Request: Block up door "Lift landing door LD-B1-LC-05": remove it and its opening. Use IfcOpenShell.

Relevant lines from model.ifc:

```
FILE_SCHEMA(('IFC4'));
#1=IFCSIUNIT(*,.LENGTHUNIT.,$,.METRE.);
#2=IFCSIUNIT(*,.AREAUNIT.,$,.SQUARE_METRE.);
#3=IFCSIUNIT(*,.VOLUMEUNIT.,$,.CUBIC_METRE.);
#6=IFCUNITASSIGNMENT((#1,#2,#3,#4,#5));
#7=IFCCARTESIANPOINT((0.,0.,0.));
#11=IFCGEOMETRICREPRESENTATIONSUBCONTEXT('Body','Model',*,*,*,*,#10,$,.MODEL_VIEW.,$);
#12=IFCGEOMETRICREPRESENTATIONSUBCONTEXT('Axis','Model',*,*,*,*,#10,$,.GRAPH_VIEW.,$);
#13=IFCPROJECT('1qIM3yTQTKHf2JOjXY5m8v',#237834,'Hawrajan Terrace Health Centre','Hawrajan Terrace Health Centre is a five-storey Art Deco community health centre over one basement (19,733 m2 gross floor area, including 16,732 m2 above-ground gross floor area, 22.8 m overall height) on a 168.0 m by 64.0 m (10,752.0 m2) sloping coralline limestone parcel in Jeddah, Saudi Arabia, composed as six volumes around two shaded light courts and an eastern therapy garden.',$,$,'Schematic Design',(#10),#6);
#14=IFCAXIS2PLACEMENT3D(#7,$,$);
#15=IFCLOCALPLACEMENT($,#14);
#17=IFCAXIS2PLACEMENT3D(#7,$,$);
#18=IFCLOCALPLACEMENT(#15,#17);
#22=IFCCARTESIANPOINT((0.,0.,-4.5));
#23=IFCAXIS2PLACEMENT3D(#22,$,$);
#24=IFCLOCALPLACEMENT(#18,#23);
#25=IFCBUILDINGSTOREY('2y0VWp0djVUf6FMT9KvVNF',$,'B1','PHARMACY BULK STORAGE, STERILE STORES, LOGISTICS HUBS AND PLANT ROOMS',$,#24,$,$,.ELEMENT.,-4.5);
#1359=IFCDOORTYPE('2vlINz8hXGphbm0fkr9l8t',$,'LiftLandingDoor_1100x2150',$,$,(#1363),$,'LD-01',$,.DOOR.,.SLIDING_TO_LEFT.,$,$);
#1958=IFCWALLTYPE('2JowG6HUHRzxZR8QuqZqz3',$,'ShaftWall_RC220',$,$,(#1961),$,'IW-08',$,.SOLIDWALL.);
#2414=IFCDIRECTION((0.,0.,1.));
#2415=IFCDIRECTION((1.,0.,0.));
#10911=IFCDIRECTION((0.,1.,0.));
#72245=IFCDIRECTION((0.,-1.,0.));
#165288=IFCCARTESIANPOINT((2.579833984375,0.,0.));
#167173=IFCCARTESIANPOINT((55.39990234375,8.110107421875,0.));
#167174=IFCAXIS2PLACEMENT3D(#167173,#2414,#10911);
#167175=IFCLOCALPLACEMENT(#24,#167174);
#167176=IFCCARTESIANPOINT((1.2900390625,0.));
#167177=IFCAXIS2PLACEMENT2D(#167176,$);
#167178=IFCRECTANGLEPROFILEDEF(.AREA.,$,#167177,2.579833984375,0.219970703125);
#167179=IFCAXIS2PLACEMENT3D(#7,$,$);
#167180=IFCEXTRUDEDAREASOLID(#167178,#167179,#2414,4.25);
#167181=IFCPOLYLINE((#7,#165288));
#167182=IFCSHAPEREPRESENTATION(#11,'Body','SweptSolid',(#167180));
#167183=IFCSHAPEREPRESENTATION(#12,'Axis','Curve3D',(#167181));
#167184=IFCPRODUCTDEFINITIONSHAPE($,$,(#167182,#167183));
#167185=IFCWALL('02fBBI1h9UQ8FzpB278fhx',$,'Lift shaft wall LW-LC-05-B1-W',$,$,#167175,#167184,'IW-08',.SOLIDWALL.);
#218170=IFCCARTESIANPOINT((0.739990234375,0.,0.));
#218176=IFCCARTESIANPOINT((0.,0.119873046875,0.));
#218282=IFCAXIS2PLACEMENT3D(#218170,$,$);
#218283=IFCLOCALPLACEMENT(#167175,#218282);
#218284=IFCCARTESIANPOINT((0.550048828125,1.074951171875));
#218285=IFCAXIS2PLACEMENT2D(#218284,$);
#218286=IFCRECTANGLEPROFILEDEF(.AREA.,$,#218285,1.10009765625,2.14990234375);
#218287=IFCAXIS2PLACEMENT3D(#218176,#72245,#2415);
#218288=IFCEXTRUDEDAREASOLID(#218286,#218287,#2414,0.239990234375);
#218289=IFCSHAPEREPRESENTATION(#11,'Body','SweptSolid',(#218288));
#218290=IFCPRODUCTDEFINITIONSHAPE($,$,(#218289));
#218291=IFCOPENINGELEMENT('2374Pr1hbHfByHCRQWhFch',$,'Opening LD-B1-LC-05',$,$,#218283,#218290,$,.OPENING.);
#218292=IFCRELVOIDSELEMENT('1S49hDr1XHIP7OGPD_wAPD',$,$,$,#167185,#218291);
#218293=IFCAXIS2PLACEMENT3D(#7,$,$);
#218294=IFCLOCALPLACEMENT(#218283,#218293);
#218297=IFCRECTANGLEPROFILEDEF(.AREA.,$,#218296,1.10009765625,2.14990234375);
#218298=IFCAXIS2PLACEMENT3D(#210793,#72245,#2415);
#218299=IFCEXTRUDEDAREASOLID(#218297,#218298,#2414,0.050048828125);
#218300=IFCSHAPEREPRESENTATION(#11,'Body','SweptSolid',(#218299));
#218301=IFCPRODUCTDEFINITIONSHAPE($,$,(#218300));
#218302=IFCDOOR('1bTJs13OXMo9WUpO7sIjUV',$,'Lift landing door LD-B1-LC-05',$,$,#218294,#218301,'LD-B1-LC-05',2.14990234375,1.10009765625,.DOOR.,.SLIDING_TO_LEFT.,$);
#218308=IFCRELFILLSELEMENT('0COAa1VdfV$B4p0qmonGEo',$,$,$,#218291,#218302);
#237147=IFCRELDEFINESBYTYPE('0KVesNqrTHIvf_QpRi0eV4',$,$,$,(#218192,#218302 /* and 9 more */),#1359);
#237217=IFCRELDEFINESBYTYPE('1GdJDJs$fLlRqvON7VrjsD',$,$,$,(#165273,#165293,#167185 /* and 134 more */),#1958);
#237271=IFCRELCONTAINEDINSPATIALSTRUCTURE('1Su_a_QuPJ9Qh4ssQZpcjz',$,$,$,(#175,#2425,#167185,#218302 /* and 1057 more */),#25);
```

```python
import ifcopenshell
import ifcopenshell.api.feature
import ifcopenshell.api.root
import ifcopenshell.geom
import ifcopenshell.util.shape

model = ifcopenshell.open("model.ifc")
settings = ifcopenshell.geom.settings()


def volume(element):
    """Net volume in cubic metres, openings subtracted."""
    shape = ifcopenshell.geom.create_shape(settings, element)
    return ifcopenshell.util.shape.get_volume(shape.geometry)


door = model.by_id(218302)
opening = door.FillsVoids[0].RelatingOpeningElement
wall = opening.VoidsElements[0].RelatingBuildingElement
before = volume(wall)

ifcopenshell.api.root.remove_product(model, product=door)
ifcopenshell.api.feature.remove_feature(model, feature=opening)

after = volume(wall)

print(f"wall volume {before:.3f} -> {after:.3f} m3")

model.write("model_v2.ifc")
```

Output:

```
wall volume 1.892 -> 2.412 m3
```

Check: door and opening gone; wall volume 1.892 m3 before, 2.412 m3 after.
